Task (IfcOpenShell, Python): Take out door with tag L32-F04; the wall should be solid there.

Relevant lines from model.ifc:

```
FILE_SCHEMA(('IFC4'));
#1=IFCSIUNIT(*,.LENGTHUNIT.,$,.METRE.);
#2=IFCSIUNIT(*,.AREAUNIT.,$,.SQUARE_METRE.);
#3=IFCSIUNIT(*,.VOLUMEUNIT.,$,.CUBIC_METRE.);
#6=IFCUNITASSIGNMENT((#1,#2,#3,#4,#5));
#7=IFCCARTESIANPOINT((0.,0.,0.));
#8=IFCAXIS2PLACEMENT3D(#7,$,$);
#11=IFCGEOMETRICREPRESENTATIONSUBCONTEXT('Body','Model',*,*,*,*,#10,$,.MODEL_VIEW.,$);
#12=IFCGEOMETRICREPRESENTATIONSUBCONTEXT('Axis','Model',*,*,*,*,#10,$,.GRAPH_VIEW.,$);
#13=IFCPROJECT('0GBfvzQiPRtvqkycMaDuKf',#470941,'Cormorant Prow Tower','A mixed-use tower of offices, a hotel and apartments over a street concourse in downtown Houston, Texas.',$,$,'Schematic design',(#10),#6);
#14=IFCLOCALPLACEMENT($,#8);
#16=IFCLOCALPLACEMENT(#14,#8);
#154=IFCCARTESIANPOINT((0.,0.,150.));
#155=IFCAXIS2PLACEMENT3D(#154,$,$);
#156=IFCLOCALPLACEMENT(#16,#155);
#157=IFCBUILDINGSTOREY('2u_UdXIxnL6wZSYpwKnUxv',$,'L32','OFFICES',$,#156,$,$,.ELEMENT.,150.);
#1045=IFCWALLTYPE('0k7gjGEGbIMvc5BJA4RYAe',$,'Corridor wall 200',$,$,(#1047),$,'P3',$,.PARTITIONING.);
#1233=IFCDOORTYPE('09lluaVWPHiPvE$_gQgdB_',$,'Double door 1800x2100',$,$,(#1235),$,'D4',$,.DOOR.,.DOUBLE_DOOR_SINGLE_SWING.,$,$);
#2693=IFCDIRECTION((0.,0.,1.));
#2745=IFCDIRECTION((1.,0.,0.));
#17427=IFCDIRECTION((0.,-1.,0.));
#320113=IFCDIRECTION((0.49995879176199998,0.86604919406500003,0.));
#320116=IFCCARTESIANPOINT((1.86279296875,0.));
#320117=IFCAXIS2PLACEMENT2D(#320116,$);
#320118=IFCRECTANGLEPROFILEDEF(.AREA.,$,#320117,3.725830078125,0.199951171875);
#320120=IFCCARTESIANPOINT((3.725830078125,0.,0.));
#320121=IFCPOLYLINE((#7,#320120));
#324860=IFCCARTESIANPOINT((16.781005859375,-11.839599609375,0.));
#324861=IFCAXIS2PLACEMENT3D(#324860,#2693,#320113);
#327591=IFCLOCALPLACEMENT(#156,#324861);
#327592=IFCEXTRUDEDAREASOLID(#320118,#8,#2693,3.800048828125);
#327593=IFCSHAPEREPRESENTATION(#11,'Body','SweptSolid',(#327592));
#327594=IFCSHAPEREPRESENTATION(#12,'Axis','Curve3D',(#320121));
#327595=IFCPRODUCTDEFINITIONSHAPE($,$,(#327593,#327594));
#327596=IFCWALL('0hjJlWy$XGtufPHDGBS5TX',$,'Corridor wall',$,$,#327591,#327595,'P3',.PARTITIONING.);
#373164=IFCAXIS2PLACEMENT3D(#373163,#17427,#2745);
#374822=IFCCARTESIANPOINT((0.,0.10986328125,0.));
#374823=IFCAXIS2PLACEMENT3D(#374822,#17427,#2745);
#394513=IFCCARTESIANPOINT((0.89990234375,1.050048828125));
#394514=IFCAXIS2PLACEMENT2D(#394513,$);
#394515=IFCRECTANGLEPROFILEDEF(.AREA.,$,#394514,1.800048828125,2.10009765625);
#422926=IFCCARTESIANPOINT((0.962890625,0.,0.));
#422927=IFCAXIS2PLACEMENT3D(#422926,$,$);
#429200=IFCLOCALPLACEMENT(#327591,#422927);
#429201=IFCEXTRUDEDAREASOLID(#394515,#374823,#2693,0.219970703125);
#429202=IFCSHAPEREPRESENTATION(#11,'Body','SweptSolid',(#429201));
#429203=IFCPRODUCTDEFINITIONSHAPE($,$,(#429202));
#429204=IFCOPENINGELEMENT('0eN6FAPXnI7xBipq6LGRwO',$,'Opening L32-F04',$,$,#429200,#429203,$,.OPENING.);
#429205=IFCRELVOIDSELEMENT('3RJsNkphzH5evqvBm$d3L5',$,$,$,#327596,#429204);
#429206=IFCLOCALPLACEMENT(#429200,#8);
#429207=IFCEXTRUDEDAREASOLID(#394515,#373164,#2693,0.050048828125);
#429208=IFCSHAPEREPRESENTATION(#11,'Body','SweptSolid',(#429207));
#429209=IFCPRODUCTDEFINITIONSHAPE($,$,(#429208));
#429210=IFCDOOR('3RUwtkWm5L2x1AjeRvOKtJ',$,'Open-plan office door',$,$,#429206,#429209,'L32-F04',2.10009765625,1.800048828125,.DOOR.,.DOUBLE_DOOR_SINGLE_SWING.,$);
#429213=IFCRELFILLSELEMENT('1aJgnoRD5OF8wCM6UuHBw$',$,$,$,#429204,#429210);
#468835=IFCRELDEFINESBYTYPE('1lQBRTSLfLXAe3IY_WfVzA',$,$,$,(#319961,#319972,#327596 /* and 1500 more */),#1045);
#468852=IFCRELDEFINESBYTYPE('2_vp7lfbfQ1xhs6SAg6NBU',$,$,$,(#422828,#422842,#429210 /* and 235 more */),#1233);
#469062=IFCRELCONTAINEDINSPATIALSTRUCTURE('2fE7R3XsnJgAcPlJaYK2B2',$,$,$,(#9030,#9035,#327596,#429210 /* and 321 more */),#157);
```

```python
import ifcopenshell
import ifcopenshell.api.feature
import ifcopenshell.api.root
import ifcopenshell.geom
import ifcopenshell.util.shape

model = ifcopenshell.open("model.ifc")
settings = ifcopenshell.geom.settings()


def volume(element):
    """Net volume in cubic metres, openings subtracted."""
    shape = ifcopenshell.geom.create_shape(settings, element)
    return ifcopenshell.util.shape.get_volume(shape.geometry)


door = model.by_guid("3RUwtkWm5L2x1AjeRvOKtJ")
opening = door.FillsVoids[0].RelatingOpeningElement
wall = opening.VoidsElements[0].RelatingBuildingElement
before = volume(wall)

ifcopenshell.api.root.remove_product(model, product=door)
ifcopenshell.api.feature.remove_feature(model, feature=opening)

after = volume(wall)

print(f"wall volume {before:.3f} -> {after:.3f} m3")

model.write("model_v2.ifc")
```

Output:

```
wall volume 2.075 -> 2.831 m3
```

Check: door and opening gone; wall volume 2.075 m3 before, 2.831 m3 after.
